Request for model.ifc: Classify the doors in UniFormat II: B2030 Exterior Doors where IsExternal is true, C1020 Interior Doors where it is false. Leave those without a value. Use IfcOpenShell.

First a look at what the model holds.

```python
import ifcopenshell
import ifcopenshell.util.element

model = ifcopenshell.open("model.ifc")
print(model.schema)
print("classifications:", [c.Name for c in model.by_type("IfcClassification")])
values = [ifcopenshell.util.element.get_pset(e, "Pset_DoorCommon", "IsExternal") for e in model.by_type("IfcDoor")]
for value in (True, False, None):
    print("IsExternal", value, values.count(value))
```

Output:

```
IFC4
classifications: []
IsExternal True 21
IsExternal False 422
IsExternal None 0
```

```python
import ifcopenshell
import ifcopenshell.api.classification
import ifcopenshell.util.element

model = ifcopenshell.open("model.ifc")

system = ifcopenshell.api.classification.add_classification(model, classification="UniFormat II")

doors = model.by_type("IfcDoor")
external = {e: ifcopenshell.util.element.get_pset(e, "Pset_DoorCommon", "IsExternal") for e in doors}
for flag, code, name in ((True, "B2030", "Exterior Doors"), (False, "C1020", "Interior Doors")):
    products = [e for e in doors if external[e] is flag]
    ifcopenshell.api.classification.add_reference(
        model, products=products, classification=system, identification=code, name=name
    )
    print(code, len(products))

model.write("model_rev.ifc")
```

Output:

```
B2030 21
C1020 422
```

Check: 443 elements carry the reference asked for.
